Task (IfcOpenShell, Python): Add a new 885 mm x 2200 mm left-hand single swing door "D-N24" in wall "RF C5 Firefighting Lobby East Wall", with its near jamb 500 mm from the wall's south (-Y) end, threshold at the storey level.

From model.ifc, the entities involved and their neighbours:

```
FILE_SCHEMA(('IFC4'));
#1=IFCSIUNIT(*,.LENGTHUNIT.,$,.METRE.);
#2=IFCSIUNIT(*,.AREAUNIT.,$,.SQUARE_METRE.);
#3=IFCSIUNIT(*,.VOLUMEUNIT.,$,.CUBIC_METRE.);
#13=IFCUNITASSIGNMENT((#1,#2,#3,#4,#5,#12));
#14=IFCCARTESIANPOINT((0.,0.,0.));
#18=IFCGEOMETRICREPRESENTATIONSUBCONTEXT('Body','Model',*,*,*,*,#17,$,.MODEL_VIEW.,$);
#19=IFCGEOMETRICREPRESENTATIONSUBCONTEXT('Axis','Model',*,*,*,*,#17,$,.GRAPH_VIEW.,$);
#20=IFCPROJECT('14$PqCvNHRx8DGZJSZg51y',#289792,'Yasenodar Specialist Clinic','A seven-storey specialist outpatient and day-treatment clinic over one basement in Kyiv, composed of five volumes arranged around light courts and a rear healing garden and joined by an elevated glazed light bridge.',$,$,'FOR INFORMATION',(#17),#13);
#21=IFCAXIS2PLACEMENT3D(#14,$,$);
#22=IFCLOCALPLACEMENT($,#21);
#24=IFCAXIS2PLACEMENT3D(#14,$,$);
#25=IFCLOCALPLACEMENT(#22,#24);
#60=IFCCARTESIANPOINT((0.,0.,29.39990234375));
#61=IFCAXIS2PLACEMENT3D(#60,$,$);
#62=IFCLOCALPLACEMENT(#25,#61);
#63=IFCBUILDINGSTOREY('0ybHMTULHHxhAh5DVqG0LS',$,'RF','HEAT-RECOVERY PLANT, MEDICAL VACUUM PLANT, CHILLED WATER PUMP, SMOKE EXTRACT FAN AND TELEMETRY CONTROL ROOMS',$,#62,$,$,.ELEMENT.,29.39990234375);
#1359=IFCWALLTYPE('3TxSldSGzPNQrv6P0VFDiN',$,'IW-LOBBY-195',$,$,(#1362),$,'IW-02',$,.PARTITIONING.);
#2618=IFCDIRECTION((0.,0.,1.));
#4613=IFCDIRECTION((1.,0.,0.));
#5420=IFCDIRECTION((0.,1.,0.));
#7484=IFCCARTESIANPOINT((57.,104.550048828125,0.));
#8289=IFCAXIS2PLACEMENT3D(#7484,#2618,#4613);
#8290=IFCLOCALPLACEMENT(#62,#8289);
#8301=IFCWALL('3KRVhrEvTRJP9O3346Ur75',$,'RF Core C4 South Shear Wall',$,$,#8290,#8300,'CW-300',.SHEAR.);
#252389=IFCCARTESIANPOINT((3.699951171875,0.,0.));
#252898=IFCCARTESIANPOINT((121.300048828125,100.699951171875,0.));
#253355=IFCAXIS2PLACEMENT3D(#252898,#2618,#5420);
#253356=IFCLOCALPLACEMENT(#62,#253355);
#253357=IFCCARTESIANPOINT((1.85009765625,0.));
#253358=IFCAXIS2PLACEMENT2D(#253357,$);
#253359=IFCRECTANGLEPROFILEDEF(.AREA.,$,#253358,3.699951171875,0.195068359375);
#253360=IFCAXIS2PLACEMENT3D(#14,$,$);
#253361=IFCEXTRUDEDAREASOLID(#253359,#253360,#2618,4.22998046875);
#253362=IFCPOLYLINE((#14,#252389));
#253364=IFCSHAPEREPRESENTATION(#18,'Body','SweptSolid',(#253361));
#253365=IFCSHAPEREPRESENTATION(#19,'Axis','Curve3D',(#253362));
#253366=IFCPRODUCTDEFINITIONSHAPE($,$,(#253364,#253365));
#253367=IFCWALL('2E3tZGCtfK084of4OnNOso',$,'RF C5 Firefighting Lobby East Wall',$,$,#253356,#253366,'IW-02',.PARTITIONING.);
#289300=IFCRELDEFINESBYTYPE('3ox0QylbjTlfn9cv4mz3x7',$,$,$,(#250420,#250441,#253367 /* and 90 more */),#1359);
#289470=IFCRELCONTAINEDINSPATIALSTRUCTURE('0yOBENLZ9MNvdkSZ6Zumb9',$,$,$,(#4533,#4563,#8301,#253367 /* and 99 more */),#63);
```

```python
import numpy as np
import ifcopenshell
import ifcopenshell.api.feature
import ifcopenshell.api.geometry
import ifcopenshell.api.root
import ifcopenshell.api.spatial
import ifcopenshell.geom
import ifcopenshell.util.element
import ifcopenshell.util.placement
import ifcopenshell.util.representation
import ifcopenshell.util.shape
import ifcopenshell.util.unit

model = ifcopenshell.open("model.ifc")
unit_scale = ifcopenshell.util.unit.calculate_unit_scale(model)
settings = ifcopenshell.geom.settings()


def volume(element):
    """Net volume in cubic metres, openings subtracted."""
    shape = ifcopenshell.geom.create_shape(settings, element)
    return ifcopenshell.util.shape.get_volume(shape.geometry)


wall = model.by_guid("2E3tZGCtfK084of4OnNOso")
storey = ifcopenshell.util.element.get_container(wall, ifc_class="IfcBuildingStorey")
context = ifcopenshell.util.representation.get_context(model, "Model", "Body", "MODEL_VIEW")
before = volume(wall)

width, height, from_end, sill = 0.885, 2.2, 0.5, 0.0  # metres

# The wall runs along its own X axis, and the end named is its -X end.
wall_shape = ifcopenshell.geom.create_shape(settings, wall)
x, y, z = ifcopenshell.util.shape.get_vertices(wall_shape.geometry).T
start = x.min() + from_end
face, thickness = float(y.min()), float(y.max() - y.min())
wall_matrix = ifcopenshell.util.placement.get_local_placement(wall.ObjectPlacement)
level = ifcopenshell.util.placement.get_local_placement(storey.ObjectPlacement)[2, 3]


def in_wall(x, y):
    """Placement at x, y metres in the wall's axes, at sill height."""
    matrix = wall_matrix.copy()
    matrix[:, 3] = wall_matrix @ np.array([x / unit_scale, y / unit_scale, 0.0, 1.0])
    matrix[2, 3] = level + sill / unit_scale
    return matrix


# Opening: a box that overshoots both wall faces by 50 mm.
opening = ifcopenshell.api.root.create_entity(model, ifc_class="IfcOpeningElement", predefined_type="OPENING")
box = ifcopenshell.api.geometry.add_wall_representation(
    model, context=context, length=width, height=height, thickness=thickness + 0.1
)
ifcopenshell.api.geometry.assign_representation(model, product=opening, representation=box)
ifcopenshell.api.geometry.edit_object_placement(model, product=opening, matrix=in_wall(start, face - 0.05), is_si=False)
ifcopenshell.api.feature.add_feature(model, feature=opening, element=wall)

door = ifcopenshell.api.root.create_entity(model, ifc_class="IfcDoor", name="D-N24", predefined_type="DOOR")
door.OverallWidth, door.OverallHeight = width / unit_scale, height / unit_scale
door.OperationType = "SINGLE_SWING_LEFT"
body = ifcopenshell.api.geometry.add_door_representation(
    model,
    context=context,
    overall_width=door.OverallWidth,
    overall_height=door.OverallHeight,
    operation_type="SINGLE_SWING_LEFT",
    lining_properties={"LiningDepth": thickness / unit_scale, "ThresholdDepth": thickness / unit_scale},
)
ifcopenshell.api.geometry.assign_representation(model, product=door, representation=body)
ifcopenshell.api.spatial.assign_container(model, products=[door], relating_structure=storey)
ifcopenshell.api.feature.add_filling(model, opening=opening, element=door)

# The lining spans the wall, so the door starts at the wall face.
ifcopenshell.api.geometry.edit_object_placement(model, product=door, matrix=in_wall(start, face), is_si=False)

after = volume(wall)

print(f"wall volume {before:.3f} -> {after:.3f} m3")

model.write("model_updated.ifc")
```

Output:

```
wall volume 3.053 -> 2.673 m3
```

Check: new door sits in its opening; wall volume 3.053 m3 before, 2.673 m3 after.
